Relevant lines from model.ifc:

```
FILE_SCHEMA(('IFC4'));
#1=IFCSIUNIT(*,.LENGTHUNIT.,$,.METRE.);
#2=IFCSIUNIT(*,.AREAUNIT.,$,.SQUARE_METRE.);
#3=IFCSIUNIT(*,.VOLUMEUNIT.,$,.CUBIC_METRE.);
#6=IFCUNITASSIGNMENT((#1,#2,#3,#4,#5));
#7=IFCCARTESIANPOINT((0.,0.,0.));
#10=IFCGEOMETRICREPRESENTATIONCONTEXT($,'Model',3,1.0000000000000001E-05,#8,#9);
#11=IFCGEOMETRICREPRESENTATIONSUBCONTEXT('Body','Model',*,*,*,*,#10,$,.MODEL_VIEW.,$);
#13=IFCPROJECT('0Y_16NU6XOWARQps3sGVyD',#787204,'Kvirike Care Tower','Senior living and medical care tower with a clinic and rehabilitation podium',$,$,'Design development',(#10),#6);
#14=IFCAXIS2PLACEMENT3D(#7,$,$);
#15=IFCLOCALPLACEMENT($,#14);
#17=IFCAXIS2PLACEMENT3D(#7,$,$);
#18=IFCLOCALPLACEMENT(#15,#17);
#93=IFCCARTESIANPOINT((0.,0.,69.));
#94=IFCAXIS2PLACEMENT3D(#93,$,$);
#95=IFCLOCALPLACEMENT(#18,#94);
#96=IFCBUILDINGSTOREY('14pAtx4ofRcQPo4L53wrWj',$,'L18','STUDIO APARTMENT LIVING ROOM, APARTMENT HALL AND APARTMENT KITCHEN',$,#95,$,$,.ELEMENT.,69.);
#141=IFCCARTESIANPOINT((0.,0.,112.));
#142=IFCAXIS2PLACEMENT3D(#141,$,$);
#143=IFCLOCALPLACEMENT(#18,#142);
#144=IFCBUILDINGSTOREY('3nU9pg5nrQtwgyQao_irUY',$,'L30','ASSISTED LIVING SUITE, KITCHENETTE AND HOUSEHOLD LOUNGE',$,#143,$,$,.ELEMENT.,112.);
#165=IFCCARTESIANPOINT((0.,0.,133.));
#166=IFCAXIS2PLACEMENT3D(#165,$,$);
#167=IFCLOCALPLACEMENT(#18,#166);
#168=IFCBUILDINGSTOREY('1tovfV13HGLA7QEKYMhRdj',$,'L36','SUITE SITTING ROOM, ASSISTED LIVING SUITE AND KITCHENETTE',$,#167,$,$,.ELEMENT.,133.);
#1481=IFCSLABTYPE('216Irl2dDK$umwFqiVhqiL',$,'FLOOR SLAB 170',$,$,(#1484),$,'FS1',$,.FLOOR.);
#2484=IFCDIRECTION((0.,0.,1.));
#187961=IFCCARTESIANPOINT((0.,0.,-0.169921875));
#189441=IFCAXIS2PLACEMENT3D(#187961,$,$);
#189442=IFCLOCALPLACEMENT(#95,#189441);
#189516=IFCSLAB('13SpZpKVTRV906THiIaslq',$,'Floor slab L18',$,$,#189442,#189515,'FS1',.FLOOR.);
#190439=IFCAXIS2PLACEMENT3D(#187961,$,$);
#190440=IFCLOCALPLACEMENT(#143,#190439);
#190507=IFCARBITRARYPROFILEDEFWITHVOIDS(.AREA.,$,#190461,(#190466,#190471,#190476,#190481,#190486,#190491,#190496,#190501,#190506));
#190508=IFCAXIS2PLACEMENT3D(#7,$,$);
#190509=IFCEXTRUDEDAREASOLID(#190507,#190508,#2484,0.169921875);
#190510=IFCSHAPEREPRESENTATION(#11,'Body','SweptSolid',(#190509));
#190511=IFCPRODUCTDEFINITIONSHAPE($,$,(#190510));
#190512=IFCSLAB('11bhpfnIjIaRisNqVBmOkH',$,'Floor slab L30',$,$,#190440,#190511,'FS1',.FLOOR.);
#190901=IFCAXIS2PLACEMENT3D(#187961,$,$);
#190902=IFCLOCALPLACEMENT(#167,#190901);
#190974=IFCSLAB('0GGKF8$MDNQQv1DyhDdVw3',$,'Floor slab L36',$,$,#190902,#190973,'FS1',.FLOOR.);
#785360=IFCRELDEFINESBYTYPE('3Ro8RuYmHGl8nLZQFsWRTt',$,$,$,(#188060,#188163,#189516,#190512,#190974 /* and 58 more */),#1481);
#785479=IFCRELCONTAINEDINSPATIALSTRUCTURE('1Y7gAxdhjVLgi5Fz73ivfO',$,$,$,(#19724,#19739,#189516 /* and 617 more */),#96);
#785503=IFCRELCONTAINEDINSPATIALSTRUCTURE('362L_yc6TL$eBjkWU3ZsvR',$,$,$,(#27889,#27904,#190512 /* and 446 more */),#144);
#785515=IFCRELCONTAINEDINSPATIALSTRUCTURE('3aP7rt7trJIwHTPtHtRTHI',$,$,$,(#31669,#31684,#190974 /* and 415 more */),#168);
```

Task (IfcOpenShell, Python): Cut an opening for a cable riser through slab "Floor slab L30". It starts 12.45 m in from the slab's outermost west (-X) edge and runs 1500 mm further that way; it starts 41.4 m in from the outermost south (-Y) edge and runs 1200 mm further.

```python
import numpy as np
import ifcopenshell
import ifcopenshell.api.feature
import ifcopenshell.api.geometry
import ifcopenshell.api.root
import ifcopenshell.geom
import ifcopenshell.util.placement
import ifcopenshell.util.representation
import ifcopenshell.util.shape
import ifcopenshell.util.unit

model = ifcopenshell.open("model.ifc")
unit_scale = ifcopenshell.util.unit.calculate_unit_scale(model)
settings = ifcopenshell.geom.settings()


def volume(element):
    """Net volume in cubic metres, openings subtracted."""
    shape = ifcopenshell.geom.create_shape(settings, element)
    return ifcopenshell.util.shape.get_volume(shape.geometry)


slab = model.by_guid("11bhpfnIjIaRisNqVBmOkH")
before = volume(slab)

# Extent in the slab's own axes, in metres. The edges named are its -X and -Y sides.
slab_shape = ifcopenshell.geom.create_shape(settings, slab)
vertices = ifcopenshell.util.shape.get_vertices(slab_shape.geometry)
x_min, y_min, bottom = vertices.min(axis=0)
top = vertices[:, 2].max()

opening = ifcopenshell.api.root.create_entity(model, ifc_class="IfcOpeningElement", name="Cable riser opening", predefined_type="OPENING")
context = ifcopenshell.util.representation.get_context(model, "Model", "Body", "MODEL_VIEW")
width, depth = 1.5, 1.2
outline = [(0.0, 0.0), (width, 0.0), (width, depth), (0.0, depth), (0.0, 0.0)]
# Overshoot both faces by 50 mm so the cut is clean.
shape = ifcopenshell.api.geometry.add_slab_representation(
    model, context=context, depth=top - bottom + 0.1, polyline=outline
)
ifcopenshell.api.geometry.assign_representation(model, product=opening, representation=shape)

matrix = ifcopenshell.util.placement.get_local_placement(slab.ObjectPlacement)
matrix[:, 3] = matrix @ np.append(np.array([x_min + 12.45, y_min + 41.4, bottom - 0.05]) / unit_scale, 1.0)
ifcopenshell.api.geometry.edit_object_placement(model, product=opening, matrix=matrix, is_si=False)
ifcopenshell.api.feature.add_feature(model, feature=opening, element=slab)

after = volume(slab)

print(f"slab volume {before:.3f} -> {after:.3f} m3")

model.write("model_v2.ifc")
```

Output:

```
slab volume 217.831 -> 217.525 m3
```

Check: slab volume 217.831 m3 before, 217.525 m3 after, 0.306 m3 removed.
